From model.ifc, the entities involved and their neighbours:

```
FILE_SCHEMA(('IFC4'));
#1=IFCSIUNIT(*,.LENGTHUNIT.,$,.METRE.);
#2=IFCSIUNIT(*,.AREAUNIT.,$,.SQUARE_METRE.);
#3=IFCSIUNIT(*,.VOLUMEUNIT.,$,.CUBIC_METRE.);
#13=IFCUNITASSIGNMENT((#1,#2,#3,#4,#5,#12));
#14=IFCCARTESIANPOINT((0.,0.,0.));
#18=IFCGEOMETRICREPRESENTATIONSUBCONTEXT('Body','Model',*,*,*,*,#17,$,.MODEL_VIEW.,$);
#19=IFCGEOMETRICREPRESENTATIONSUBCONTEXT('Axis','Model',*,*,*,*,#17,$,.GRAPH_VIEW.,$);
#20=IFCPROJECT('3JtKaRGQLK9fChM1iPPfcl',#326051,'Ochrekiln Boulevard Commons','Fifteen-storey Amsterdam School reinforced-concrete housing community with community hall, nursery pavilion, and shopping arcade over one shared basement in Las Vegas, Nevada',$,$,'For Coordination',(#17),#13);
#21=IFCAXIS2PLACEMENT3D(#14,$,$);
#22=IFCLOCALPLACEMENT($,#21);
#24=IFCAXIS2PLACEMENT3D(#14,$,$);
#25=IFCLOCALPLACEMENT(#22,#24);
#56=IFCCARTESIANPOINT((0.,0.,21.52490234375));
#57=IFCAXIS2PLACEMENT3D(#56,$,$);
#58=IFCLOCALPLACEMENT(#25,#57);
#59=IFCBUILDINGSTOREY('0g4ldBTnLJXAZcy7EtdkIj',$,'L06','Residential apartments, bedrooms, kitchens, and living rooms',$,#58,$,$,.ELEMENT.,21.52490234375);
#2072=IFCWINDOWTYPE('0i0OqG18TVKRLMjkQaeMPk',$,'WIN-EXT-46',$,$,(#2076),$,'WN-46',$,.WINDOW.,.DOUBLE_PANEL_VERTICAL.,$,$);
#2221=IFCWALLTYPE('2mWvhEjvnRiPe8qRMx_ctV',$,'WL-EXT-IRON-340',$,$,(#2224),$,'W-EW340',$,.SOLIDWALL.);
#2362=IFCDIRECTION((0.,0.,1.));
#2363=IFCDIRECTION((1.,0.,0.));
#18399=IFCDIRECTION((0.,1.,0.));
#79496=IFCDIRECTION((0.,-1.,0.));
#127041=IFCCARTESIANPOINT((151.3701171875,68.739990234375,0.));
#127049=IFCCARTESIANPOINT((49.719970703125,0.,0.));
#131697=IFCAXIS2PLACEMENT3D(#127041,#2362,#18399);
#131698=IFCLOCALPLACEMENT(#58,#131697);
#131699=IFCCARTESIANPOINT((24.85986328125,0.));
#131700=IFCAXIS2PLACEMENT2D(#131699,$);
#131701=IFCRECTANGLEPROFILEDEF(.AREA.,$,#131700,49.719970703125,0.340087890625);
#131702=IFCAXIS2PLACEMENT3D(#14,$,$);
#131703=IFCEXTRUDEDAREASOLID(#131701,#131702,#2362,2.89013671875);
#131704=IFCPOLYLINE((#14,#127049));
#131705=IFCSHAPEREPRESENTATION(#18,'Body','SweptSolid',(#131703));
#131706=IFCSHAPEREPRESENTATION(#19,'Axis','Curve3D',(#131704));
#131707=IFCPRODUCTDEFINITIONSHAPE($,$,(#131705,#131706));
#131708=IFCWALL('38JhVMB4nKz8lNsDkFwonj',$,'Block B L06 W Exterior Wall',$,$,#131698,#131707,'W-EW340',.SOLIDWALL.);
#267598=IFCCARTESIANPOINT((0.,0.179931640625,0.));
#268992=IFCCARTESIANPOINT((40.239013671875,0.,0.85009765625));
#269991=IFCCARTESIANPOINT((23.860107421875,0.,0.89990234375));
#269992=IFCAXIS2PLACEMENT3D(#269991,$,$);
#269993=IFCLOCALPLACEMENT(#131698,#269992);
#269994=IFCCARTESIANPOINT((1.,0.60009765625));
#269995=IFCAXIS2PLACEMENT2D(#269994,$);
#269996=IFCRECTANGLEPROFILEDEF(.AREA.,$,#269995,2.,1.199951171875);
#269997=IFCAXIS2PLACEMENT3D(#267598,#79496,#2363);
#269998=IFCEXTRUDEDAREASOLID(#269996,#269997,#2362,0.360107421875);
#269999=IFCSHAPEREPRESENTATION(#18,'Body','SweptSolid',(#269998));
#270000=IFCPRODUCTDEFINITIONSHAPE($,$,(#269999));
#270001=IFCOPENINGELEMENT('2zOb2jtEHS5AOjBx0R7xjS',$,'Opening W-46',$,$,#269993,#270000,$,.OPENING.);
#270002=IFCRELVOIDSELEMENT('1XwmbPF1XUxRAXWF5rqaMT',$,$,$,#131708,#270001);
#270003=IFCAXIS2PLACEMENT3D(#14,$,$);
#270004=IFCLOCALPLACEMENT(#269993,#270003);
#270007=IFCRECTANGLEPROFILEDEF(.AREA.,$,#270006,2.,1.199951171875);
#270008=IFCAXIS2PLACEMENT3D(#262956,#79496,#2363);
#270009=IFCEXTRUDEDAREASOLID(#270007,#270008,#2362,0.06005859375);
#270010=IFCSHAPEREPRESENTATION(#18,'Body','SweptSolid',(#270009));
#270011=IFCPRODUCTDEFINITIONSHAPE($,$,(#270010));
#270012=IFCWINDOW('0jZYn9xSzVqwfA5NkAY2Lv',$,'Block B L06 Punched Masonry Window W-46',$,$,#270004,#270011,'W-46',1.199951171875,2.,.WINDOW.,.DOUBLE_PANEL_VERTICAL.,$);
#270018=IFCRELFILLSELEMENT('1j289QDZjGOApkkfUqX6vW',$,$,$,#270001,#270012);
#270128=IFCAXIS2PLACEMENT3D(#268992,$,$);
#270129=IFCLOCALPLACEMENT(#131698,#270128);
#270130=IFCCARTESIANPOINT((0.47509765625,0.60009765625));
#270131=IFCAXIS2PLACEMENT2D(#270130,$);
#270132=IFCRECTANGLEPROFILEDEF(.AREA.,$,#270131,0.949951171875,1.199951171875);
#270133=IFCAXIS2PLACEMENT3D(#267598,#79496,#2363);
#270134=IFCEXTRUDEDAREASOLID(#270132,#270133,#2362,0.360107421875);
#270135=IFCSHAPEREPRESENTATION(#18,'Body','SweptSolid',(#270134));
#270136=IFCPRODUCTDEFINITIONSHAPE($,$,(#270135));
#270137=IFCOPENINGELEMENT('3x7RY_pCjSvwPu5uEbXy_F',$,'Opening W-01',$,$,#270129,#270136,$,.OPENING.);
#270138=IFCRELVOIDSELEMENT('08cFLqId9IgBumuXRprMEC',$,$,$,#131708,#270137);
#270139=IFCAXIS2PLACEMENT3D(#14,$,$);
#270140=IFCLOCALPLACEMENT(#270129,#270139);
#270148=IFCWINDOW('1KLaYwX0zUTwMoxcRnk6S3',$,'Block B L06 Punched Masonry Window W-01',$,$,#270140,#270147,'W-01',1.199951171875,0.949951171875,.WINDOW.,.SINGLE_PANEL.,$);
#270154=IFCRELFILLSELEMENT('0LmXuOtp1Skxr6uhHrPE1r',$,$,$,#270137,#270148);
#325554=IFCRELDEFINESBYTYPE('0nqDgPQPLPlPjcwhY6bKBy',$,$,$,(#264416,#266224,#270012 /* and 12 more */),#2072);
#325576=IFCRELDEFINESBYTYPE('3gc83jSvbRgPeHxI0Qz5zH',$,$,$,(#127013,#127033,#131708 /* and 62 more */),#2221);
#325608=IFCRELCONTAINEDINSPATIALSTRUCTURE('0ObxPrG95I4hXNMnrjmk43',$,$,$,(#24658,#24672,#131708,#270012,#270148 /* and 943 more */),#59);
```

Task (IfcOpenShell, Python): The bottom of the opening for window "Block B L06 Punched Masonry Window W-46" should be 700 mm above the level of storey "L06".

```python
import numpy as np
import ifcopenshell
import ifcopenshell.api.geometry
import ifcopenshell.geom
import ifcopenshell.util.element
import ifcopenshell.util.placement
import ifcopenshell.util.shape
import ifcopenshell.util.unit

model = ifcopenshell.open("model.ifc")
unit_scale = ifcopenshell.util.unit.calculate_unit_scale(model)

window = model.by_guid("0jZYn9xSzVqwfA5NkAY2Lv")
opening = window.FillsVoids[0].RelatingOpeningElement
storey = ifcopenshell.util.element.get_container(window, ifc_class="IfcBuildingStorey")
level = ifcopenshell.util.placement.get_local_placement(storey.ObjectPlacement)[2, 3]

# The opening's origin need not be at the sill, so measure its lowest point.
shape = ifcopenshell.geom.create_shape(ifcopenshell.geom.settings(), opening)
bottom = ifcopenshell.util.shape.get_shape_bottom_elevation(shape, shape.geometry) / unit_scale
dz = level + 0.7 / unit_scale - bottom

shift = np.array([0.0, 0.0, dz])
# The window is placed relative to its opening, so it follows when the opening moves.
matrix = ifcopenshell.util.placement.get_local_placement(opening.ObjectPlacement)
matrix[:3, 3] += shift
ifcopenshell.api.geometry.edit_object_placement(
    model, product=opening, matrix=matrix, is_si=False, should_transform_children=True
)

print(f"moved by {dz * unit_scale:+.3f} m")

model.write("model_edited.ifc")
```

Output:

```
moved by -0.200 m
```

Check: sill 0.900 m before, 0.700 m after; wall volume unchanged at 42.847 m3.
